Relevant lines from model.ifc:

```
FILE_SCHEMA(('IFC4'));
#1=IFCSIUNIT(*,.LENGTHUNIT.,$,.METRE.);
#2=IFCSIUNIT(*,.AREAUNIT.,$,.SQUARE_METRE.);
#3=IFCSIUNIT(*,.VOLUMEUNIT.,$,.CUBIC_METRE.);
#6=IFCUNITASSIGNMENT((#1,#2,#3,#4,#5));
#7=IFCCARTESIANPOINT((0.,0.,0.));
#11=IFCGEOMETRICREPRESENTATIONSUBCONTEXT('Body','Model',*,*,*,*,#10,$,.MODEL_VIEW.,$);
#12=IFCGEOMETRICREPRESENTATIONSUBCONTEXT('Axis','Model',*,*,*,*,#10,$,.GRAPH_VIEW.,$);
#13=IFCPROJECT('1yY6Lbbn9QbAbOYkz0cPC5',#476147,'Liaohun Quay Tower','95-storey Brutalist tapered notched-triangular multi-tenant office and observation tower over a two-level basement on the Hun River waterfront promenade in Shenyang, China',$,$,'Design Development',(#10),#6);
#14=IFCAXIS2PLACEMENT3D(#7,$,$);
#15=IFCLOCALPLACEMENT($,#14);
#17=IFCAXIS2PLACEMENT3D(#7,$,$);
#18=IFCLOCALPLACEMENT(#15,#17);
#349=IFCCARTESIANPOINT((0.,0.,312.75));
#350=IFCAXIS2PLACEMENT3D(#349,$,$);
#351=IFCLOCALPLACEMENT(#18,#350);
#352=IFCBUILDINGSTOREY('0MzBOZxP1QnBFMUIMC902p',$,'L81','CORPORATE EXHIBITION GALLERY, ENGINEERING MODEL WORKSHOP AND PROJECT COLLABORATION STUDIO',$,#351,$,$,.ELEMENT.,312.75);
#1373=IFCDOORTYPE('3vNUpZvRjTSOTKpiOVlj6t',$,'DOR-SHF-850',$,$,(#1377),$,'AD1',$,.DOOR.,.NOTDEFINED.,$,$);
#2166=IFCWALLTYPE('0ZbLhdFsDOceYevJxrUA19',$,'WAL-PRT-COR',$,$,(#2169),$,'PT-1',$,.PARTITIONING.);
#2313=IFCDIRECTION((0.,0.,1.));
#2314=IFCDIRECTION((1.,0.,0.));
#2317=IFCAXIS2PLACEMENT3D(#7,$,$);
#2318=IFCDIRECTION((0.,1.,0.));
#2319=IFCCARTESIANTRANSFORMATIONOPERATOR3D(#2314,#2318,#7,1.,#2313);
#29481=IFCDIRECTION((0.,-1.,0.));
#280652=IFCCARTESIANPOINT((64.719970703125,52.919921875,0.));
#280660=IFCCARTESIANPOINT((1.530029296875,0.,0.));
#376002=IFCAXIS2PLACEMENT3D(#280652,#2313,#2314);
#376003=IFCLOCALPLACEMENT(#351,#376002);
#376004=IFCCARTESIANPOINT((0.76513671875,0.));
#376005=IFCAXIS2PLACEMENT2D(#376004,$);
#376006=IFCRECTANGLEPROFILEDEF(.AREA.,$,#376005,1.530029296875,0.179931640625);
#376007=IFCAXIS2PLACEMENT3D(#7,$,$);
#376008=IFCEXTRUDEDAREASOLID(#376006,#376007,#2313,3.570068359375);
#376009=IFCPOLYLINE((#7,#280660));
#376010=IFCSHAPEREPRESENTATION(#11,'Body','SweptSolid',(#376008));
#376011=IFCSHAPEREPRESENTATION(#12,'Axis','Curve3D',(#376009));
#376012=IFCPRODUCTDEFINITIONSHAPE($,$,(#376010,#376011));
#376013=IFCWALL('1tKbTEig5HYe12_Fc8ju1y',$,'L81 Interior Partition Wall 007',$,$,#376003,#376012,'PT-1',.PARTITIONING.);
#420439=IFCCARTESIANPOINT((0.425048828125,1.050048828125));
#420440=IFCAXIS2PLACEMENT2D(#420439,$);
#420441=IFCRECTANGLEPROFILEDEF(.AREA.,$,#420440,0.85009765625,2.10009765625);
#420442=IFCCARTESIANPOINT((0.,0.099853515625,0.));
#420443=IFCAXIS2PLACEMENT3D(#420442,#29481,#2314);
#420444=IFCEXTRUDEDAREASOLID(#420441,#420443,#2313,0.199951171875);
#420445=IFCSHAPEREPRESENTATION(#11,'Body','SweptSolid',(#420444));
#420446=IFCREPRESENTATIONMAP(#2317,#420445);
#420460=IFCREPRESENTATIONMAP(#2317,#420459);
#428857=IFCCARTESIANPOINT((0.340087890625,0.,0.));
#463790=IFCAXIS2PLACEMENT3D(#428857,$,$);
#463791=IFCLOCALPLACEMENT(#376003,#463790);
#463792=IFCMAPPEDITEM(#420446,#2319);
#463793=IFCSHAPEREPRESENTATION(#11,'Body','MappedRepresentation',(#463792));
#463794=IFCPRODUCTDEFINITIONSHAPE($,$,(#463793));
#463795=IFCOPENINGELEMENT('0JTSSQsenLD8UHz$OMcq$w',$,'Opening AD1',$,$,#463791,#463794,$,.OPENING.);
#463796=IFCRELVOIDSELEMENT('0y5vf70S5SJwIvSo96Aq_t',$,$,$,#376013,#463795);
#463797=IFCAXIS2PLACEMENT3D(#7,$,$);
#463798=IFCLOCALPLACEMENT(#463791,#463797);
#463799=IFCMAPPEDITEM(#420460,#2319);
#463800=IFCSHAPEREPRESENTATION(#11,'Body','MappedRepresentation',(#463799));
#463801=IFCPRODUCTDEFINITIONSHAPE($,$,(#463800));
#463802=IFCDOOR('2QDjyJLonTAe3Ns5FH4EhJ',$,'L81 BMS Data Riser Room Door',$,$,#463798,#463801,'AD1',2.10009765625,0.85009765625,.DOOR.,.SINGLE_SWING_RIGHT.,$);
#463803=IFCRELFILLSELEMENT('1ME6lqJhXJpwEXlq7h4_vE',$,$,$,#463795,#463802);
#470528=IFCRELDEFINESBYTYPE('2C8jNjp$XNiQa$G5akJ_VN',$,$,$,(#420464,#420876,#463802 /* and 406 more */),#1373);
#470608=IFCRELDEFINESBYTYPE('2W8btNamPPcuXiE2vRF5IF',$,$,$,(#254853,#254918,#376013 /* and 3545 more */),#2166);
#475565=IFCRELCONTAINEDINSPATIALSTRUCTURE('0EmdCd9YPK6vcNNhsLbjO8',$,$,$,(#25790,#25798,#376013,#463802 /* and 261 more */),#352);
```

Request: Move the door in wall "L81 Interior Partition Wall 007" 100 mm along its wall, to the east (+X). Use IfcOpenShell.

```python
import ifcopenshell
import ifcopenshell.api.geometry
import ifcopenshell.util.placement
import ifcopenshell.util.unit

model = ifcopenshell.open("model.ifc")
unit_scale = ifcopenshell.util.unit.calculate_unit_scale(model)

door = model.by_id(463802)
opening = door.FillsVoids[0].RelatingOpeningElement
wall = opening.VoidsElements[0].RelatingBuildingElement

wall_matrix = ifcopenshell.util.placement.get_local_placement(wall.ObjectPlacement)
shift = wall_matrix[:3, 0] * 0.1 / unit_scale
before = ifcopenshell.util.placement.get_local_placement(door.ObjectPlacement)[:3, 3].copy()

# The door is placed relative to its opening, so it follows when the opening moves.
matrix = ifcopenshell.util.placement.get_local_placement(opening.ObjectPlacement)
matrix[:3, 3] += shift
ifcopenshell.api.geometry.edit_object_placement(
    model, product=opening, matrix=matrix, is_si=False, should_transform_children=True
)

after = ifcopenshell.util.placement.get_local_placement(door.ObjectPlacement)[:3, 3]
print("door moved by", (after - before).round(3) + 0.0)

model.write("model_edited.ifc")
```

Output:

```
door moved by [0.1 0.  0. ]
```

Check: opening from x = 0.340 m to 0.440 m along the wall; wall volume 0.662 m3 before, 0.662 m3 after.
